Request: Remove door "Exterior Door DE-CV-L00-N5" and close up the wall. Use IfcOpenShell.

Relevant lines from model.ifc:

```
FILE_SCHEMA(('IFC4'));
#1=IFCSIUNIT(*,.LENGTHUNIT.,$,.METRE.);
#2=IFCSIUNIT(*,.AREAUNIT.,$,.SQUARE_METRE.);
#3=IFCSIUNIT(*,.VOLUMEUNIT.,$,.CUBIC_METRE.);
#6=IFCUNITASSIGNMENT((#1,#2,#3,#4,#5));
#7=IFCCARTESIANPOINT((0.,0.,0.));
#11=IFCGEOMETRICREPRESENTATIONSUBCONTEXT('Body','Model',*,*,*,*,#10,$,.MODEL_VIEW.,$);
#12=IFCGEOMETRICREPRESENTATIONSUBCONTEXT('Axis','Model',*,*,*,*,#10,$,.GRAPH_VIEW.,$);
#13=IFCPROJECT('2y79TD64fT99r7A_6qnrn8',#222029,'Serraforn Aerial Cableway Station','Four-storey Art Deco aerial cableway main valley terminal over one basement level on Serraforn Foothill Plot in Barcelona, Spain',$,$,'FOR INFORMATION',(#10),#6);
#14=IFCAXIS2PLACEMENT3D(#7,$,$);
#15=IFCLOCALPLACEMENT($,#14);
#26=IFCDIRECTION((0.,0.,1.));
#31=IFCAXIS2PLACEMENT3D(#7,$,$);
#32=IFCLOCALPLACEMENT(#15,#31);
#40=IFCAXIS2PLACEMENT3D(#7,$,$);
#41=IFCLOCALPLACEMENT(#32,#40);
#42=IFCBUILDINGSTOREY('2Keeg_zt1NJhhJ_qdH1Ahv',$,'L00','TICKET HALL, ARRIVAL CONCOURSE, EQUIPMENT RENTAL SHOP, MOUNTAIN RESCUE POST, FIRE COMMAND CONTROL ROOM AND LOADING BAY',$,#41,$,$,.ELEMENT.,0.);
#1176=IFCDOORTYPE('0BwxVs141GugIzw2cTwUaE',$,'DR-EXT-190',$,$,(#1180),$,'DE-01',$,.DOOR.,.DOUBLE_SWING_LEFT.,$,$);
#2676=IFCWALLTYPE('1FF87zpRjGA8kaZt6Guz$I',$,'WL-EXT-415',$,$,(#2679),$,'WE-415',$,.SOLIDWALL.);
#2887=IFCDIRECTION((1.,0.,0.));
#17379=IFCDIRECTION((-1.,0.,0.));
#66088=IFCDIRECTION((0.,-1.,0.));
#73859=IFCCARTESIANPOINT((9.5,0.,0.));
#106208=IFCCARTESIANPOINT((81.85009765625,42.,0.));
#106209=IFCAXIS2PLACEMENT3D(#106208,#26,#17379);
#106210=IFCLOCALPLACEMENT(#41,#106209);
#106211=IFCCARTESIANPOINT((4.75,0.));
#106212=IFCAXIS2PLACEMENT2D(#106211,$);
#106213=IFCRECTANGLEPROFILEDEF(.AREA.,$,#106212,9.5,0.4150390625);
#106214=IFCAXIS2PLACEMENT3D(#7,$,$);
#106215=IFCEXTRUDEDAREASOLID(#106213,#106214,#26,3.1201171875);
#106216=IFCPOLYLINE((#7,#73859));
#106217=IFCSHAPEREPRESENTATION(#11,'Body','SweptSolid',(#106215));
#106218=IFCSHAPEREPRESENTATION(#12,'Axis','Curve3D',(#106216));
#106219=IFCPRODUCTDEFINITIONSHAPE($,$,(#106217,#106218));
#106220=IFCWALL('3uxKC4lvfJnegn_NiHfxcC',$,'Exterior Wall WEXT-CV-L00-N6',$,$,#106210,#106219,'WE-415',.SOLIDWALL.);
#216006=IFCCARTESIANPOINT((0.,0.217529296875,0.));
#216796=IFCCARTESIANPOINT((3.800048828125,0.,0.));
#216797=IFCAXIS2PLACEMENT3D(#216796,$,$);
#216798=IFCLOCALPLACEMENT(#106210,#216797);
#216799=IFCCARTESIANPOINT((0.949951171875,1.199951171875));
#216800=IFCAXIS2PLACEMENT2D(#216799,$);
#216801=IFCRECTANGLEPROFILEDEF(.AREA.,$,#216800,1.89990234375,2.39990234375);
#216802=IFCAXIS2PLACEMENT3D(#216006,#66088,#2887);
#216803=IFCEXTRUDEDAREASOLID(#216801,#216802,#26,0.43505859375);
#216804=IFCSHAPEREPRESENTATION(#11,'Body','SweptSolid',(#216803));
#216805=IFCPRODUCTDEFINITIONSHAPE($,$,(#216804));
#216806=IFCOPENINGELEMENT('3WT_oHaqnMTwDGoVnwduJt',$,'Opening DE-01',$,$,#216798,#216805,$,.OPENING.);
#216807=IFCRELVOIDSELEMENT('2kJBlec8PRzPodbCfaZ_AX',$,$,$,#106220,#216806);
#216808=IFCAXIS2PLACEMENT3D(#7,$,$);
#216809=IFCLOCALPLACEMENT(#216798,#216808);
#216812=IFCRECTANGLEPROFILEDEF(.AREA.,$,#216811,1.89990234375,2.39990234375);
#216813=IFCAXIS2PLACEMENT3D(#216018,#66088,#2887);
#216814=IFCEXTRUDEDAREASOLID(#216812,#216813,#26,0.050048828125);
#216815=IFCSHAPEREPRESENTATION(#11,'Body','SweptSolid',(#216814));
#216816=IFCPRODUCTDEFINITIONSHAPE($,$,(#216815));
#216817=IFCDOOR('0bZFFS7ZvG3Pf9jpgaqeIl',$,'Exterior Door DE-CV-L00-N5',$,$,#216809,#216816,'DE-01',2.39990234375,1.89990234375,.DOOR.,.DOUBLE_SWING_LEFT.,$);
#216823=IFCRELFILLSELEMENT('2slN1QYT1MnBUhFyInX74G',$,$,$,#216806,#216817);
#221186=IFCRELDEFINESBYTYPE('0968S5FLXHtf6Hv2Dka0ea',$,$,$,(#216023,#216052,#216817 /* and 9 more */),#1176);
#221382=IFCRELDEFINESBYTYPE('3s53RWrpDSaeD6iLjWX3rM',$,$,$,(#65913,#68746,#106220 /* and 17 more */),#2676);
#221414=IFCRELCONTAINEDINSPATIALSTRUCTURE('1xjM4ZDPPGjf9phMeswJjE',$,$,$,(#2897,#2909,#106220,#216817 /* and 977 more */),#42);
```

```python
import ifcopenshell
import ifcopenshell.api.feature
import ifcopenshell.api.root
import ifcopenshell.geom
import ifcopenshell.util.shape

model = ifcopenshell.open("model.ifc")
settings = ifcopenshell.geom.settings()


def volume(element):
    """Net volume in cubic metres, openings subtracted."""
    shape = ifcopenshell.geom.create_shape(settings, element)
    return ifcopenshell.util.shape.get_volume(shape.geometry)


door = model.by_id(216817)
opening = door.FillsVoids[0].RelatingOpeningElement
wall = opening.VoidsElements[0].RelatingBuildingElement
before = volume(wall)

ifcopenshell.api.root.remove_product(model, product=door)
ifcopenshell.api.feature.remove_feature(model, feature=opening)

after = volume(wall)

print(f"wall volume {before:.3f} -> {after:.3f} m3")

model.write("model_rev.ifc")
```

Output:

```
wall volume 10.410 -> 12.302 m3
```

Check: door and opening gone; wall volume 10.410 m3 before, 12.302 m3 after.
